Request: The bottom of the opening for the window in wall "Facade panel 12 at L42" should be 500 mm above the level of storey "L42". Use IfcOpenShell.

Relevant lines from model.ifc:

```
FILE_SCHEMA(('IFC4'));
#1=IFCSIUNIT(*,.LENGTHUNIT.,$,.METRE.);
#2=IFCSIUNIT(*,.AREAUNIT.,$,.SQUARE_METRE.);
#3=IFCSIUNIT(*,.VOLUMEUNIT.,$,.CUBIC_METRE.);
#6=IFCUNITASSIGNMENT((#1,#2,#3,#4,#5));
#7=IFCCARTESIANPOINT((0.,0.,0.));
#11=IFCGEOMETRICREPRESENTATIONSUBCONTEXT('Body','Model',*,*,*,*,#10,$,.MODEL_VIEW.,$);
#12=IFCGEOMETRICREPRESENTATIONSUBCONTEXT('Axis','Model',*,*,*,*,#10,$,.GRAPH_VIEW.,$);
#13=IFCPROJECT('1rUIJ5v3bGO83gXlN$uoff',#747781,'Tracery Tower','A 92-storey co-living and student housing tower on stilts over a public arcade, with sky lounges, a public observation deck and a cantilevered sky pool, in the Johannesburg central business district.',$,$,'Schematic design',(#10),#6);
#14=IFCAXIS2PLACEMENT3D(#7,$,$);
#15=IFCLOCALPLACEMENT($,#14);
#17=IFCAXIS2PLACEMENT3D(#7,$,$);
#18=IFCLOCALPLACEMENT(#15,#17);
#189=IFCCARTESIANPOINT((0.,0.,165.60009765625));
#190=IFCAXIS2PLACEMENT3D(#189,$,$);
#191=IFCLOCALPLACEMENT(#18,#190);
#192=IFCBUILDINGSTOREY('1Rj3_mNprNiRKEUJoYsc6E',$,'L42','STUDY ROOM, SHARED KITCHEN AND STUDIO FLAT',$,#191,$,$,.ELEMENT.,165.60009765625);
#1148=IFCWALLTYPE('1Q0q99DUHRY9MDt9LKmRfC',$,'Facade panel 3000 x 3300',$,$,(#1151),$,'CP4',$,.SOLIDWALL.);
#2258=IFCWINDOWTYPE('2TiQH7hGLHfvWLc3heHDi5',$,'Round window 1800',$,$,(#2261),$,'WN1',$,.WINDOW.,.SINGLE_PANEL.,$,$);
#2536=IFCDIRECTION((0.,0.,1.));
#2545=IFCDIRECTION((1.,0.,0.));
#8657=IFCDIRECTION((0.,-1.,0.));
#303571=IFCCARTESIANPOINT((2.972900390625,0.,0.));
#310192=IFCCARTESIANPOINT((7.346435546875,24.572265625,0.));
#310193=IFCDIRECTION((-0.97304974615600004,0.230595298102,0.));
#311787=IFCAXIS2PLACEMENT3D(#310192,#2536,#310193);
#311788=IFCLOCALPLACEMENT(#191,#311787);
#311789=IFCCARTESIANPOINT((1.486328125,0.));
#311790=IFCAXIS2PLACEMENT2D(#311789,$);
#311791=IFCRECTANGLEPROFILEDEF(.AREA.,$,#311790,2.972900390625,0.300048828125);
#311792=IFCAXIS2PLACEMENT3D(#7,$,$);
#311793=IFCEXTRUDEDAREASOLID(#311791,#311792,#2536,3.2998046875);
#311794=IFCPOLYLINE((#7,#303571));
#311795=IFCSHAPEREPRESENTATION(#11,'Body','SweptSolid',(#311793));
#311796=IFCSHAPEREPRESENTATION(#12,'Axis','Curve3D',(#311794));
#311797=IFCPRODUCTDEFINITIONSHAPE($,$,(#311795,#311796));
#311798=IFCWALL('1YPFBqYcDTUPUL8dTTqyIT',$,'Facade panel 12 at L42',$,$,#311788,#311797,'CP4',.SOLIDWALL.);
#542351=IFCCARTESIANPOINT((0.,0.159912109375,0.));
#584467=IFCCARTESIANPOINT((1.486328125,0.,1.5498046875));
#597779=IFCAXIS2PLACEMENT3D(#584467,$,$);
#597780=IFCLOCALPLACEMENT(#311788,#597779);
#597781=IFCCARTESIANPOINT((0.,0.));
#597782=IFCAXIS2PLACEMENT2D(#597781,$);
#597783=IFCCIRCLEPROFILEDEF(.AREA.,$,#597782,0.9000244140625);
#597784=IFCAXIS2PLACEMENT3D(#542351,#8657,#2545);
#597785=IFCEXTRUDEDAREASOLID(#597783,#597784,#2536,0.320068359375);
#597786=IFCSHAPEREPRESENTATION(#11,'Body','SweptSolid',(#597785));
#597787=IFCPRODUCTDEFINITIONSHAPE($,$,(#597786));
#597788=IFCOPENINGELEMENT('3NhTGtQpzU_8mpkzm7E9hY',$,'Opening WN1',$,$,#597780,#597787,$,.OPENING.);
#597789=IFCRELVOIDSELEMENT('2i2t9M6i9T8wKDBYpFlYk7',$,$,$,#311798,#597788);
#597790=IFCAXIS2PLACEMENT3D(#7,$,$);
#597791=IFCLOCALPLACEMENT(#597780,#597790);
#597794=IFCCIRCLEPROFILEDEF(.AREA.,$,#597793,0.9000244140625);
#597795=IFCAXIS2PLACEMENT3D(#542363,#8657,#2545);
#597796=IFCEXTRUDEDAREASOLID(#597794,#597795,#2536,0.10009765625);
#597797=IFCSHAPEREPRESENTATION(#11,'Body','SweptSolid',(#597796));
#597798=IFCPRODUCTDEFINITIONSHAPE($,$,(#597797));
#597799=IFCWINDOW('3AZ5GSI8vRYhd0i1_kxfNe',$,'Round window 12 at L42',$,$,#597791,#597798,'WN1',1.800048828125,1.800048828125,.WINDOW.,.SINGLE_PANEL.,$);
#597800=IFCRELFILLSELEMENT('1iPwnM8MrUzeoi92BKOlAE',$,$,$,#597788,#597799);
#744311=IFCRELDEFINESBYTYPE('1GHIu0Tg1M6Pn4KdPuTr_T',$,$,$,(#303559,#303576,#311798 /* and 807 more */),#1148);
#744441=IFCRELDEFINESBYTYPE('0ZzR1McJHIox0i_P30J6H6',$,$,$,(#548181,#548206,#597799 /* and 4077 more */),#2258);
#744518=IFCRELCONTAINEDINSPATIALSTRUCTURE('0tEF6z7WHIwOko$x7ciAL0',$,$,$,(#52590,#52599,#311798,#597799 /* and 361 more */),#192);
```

```python
import numpy as np
import ifcopenshell
import ifcopenshell.api.geometry
import ifcopenshell.geom
import ifcopenshell.util.element
import ifcopenshell.util.placement
import ifcopenshell.util.shape
import ifcopenshell.util.unit

model = ifcopenshell.open("model.ifc")
unit_scale = ifcopenshell.util.unit.calculate_unit_scale(model)

window = model.by_guid("3AZ5GSI8vRYhd0i1_kxfNe")
opening = window.FillsVoids[0].RelatingOpeningElement
storey = ifcopenshell.util.element.get_container(window, ifc_class="IfcBuildingStorey")
level = ifcopenshell.util.placement.get_local_placement(storey.ObjectPlacement)[2, 3]

# The opening's origin need not be at the sill, so measure its lowest point.
shape = ifcopenshell.geom.create_shape(ifcopenshell.geom.settings(), opening)
bottom = ifcopenshell.util.shape.get_shape_bottom_elevation(shape, shape.geometry) / unit_scale
dz = level + 0.5 / unit_scale - bottom

shift = np.array([0.0, 0.0, dz])
# The window is placed relative to its opening, so it follows when the opening moves.
matrix = ifcopenshell.util.placement.get_local_placement(opening.ObjectPlacement)
matrix[:3, 3] += shift
ifcopenshell.api.geometry.edit_object_placement(
    model, product=opening, matrix=matrix, is_si=False, should_transform_children=True
)

print(f"moved by {dz * unit_scale:+.3f} m")

model.write("model_v2.ifc")
```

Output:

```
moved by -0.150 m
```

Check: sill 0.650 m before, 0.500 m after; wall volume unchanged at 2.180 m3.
